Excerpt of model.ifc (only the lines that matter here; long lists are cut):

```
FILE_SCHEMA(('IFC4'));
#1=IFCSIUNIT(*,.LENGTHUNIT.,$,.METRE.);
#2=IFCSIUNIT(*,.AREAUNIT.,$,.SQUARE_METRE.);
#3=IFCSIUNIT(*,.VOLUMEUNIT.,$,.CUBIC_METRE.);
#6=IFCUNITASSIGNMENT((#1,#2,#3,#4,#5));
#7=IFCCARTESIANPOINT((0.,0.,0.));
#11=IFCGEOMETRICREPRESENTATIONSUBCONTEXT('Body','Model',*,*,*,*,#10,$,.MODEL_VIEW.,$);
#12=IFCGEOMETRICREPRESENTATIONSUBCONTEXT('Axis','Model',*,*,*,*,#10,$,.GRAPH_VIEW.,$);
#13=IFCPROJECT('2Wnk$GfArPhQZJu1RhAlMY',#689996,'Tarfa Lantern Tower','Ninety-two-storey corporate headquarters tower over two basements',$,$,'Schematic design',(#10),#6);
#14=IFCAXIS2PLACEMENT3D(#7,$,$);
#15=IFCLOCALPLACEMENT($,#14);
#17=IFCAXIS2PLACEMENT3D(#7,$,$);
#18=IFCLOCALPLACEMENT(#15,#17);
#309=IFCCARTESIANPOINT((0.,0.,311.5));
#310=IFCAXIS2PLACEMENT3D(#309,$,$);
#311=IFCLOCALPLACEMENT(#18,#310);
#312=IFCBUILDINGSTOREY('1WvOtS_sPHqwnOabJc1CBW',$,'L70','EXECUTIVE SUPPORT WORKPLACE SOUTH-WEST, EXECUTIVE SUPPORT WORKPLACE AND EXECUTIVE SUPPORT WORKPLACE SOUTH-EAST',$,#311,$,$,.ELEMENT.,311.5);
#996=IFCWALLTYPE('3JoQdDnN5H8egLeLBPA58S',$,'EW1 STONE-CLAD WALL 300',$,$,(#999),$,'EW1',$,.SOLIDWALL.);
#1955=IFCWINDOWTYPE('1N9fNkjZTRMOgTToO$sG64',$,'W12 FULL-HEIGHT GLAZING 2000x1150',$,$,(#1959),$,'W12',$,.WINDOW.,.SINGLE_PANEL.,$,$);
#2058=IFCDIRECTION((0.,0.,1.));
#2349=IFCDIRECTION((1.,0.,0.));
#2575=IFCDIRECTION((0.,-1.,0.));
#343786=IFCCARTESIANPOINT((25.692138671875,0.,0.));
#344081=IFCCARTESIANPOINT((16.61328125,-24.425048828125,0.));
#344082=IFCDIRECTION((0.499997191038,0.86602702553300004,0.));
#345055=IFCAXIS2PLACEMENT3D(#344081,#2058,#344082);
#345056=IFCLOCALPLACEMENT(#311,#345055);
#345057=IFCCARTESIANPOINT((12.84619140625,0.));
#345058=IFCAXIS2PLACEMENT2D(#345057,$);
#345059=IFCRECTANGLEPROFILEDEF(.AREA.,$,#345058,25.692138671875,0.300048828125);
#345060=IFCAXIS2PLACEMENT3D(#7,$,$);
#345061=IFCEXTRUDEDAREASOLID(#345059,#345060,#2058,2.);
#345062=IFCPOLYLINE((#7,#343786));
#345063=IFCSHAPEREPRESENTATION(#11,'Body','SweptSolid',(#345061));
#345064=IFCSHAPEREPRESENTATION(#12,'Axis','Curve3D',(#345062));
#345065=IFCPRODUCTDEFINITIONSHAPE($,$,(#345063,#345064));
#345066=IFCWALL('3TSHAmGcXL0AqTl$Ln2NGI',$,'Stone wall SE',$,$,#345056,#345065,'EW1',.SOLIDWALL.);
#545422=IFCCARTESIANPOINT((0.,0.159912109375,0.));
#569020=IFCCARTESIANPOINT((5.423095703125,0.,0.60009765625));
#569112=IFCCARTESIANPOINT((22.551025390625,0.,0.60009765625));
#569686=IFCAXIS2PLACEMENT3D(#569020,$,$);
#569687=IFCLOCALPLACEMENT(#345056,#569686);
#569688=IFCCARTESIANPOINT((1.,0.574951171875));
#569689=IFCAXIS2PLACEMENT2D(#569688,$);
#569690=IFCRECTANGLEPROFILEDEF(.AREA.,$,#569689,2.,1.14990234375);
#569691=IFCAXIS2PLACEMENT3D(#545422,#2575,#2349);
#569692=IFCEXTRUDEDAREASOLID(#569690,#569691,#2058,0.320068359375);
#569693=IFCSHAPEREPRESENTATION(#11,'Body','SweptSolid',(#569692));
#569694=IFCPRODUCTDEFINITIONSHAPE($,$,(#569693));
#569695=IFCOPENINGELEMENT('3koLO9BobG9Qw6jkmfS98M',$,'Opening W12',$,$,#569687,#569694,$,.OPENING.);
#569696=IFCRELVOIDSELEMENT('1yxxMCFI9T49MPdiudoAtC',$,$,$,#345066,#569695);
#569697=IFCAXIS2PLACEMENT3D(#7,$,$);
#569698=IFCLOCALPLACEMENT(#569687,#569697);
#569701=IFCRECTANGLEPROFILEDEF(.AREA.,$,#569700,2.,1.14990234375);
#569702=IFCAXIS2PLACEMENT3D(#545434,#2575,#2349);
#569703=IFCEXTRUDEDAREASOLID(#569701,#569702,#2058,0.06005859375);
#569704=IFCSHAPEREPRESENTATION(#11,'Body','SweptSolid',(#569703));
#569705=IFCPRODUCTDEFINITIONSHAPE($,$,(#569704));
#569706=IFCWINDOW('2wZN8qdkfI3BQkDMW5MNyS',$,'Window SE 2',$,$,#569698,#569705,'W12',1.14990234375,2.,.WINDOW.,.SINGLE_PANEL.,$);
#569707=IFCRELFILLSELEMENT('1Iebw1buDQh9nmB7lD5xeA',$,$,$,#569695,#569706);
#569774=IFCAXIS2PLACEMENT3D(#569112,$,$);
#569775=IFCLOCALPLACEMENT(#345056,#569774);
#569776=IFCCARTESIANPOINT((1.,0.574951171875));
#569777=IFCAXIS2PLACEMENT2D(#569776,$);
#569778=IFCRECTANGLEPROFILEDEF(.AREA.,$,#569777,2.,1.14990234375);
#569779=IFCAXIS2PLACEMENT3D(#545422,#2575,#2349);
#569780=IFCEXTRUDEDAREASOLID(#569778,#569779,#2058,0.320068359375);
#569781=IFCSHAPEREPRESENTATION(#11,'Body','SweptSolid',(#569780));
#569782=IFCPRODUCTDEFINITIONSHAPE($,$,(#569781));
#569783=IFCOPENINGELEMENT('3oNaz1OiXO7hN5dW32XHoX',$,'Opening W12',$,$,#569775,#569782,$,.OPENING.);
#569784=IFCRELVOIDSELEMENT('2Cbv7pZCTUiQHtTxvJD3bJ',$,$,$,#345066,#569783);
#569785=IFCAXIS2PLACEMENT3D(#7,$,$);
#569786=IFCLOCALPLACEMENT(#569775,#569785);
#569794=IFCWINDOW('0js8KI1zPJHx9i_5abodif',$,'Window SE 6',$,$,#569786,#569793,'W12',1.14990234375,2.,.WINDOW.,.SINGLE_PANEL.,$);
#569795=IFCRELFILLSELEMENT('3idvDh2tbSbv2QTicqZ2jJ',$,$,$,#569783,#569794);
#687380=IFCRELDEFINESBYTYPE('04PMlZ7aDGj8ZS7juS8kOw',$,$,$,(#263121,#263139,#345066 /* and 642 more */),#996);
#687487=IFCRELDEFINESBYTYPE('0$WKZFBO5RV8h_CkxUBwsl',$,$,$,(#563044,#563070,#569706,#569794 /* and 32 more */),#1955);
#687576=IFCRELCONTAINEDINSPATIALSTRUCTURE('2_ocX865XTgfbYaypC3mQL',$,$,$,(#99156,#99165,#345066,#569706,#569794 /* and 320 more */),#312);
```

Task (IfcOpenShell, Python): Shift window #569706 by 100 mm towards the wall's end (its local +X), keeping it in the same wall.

```python
import ifcopenshell
import ifcopenshell.api.geometry
import ifcopenshell.util.placement
import ifcopenshell.util.unit

model = ifcopenshell.open("model.ifc")
unit_scale = ifcopenshell.util.unit.calculate_unit_scale(model)

window = model.by_guid("2wZN8qdkfI3BQkDMW5MNyS")
opening = window.FillsVoids[0].RelatingOpeningElement
wall = opening.VoidsElements[0].RelatingBuildingElement

wall_matrix = ifcopenshell.util.placement.get_local_placement(wall.ObjectPlacement)
shift = wall_matrix[:3, 0] * 0.1 / unit_scale
before = ifcopenshell.util.placement.get_local_placement(window.ObjectPlacement)[:3, 3].copy()

# The window is placed relative to its opening, so it follows when the opening moves.
matrix = ifcopenshell.util.placement.get_local_placement(opening.ObjectPlacement)
matrix[:3, 3] += shift
ifcopenshell.api.geometry.edit_object_placement(
    model, product=opening, matrix=matrix, is_si=False, should_transform_children=True
)

after = ifcopenshell.util.placement.get_local_placement(window.ObjectPlacement)[:3, 3]
print("window moved by", (after - before).round(3) + 0.0)

model.write("model_updated.ifc")
```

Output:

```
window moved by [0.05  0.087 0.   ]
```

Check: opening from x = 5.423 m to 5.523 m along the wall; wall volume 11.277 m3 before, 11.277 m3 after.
